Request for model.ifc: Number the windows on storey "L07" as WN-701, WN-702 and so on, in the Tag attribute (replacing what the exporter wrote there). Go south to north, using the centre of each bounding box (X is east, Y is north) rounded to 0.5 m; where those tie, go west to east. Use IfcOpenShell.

First a look at what the model holds.

```python
import ifcopenshell
import ifcopenshell.util.element
import ifcopenshell.util.placement

model = ifcopenshell.open("model.ifc")
print(model.schema)
storey = next(s for s in model.by_type("IfcBuildingStorey") if s.Name == "L07")
windows = [e for e in ifcopenshell.util.element.get_decomposition(storey) if e.is_a("IfcWindow")]
for e in sorted(windows, key=lambda e: e.id()):
    origin = ifcopenshell.util.placement.get_local_placement(e.ObjectPlacement)[:3, 3]
    print(e.id(), e.Tag, e.Name, origin.round(2) + 0.0, sep=" | ")
```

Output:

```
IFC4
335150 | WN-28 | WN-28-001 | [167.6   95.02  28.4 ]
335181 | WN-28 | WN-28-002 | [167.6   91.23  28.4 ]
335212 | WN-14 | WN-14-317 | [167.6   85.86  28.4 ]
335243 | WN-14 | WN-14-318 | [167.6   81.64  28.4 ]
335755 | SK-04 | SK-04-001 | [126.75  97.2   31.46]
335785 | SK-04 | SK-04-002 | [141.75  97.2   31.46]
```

```python
import ifcopenshell
import ifcopenshell.geom
import ifcopenshell.util.element
import ifcopenshell.util.shape

model = ifcopenshell.open("model.ifc")
settings = ifcopenshell.geom.settings()
settings.set("use-world-coords", True)


def centre(element):
    shape = ifcopenshell.geom.create_shape(settings, element)
    return ifcopenshell.util.shape.get_bbox_centroid(shape.geometry)


storey = next(s for s in model.by_type("IfcBuildingStorey") if s.Name == "L07")
windows = [e for e in ifcopenshell.util.element.get_decomposition(storey) if e.is_a("IfcWindow")]

# Insertion points can sit at a corner or the storey origin, so sort by the geometry (in metres).
centres = {e: centre(e) for e in windows}
windows.sort(key=lambda e: (round(centres[e][1] / 0.5), centres[e][0]))

for i, e in enumerate(windows, start=1):
    number = f"WN-7{i:02d}"
    e.Tag = number
    print(e.id(), number)

model.write("model_edited.ifc")
```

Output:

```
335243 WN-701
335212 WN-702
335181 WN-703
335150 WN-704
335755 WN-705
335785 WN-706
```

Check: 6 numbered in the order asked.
